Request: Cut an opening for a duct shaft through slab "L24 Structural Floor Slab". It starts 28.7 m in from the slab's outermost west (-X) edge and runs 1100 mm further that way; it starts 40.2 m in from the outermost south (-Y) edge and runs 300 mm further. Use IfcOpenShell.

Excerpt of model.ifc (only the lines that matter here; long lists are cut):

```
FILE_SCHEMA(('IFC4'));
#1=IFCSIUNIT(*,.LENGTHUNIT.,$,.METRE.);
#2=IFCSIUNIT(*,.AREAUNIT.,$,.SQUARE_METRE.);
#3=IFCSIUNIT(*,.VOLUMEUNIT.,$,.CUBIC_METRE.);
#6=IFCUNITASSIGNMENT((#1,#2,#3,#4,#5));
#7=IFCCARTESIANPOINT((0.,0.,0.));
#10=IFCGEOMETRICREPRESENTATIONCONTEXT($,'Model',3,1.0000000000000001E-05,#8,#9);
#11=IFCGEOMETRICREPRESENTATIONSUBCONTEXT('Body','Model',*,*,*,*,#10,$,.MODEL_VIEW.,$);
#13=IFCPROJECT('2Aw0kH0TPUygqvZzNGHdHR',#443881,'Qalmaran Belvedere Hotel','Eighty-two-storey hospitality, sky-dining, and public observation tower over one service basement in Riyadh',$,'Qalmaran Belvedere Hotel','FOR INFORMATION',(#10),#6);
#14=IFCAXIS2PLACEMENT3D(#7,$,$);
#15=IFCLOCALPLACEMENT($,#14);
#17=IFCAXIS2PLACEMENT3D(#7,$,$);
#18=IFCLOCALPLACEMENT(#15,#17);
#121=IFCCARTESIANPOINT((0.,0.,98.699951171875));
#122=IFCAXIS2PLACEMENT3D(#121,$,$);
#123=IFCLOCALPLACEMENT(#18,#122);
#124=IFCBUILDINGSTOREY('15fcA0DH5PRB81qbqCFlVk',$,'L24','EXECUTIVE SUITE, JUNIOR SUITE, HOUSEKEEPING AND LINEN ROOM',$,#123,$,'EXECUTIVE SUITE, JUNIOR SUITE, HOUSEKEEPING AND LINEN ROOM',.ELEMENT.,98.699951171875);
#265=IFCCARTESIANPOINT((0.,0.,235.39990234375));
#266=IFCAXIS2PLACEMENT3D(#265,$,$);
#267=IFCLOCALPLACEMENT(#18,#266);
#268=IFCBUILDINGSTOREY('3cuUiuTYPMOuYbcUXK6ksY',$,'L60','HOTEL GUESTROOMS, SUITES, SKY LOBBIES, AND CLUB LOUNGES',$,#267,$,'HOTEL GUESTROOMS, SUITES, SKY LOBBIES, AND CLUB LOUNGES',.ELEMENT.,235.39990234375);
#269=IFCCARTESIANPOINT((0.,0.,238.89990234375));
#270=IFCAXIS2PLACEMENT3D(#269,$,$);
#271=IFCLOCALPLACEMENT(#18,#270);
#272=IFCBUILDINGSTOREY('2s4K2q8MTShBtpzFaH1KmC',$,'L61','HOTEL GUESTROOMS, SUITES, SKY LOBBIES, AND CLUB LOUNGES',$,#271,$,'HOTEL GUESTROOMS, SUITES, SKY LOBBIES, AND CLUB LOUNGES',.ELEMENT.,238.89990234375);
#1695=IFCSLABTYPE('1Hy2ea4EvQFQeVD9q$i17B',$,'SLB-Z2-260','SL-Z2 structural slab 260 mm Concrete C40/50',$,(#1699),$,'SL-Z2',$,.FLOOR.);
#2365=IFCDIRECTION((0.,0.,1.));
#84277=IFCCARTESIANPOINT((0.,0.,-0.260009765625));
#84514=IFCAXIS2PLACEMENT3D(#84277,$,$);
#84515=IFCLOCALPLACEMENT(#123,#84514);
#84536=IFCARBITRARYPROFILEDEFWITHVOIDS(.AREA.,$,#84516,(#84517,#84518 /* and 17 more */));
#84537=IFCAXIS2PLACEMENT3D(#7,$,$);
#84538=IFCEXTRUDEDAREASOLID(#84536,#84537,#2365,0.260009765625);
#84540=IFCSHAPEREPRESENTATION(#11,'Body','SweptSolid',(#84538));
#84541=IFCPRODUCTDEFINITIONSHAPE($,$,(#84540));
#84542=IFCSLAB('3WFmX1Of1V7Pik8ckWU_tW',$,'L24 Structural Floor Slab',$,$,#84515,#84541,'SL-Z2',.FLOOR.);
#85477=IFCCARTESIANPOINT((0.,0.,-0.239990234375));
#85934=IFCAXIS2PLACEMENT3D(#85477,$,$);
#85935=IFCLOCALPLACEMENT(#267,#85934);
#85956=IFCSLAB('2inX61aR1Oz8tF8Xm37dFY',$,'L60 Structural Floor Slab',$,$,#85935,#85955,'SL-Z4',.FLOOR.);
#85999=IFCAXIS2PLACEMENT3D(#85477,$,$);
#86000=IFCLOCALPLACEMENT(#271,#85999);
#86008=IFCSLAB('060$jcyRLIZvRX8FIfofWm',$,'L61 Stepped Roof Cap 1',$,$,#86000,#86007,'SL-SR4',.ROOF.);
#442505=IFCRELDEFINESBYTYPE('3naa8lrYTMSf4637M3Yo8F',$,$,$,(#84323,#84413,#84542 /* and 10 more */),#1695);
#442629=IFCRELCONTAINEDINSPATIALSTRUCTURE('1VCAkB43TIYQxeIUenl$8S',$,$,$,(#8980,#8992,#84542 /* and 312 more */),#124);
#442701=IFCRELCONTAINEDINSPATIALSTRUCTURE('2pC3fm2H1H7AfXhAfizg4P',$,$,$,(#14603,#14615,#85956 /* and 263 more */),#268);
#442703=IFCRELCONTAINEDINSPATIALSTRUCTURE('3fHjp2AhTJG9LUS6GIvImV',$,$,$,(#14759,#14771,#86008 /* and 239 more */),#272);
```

```python
import numpy as np
import ifcopenshell
import ifcopenshell.api.feature
import ifcopenshell.api.geometry
import ifcopenshell.api.root
import ifcopenshell.geom
import ifcopenshell.util.placement
import ifcopenshell.util.representation
import ifcopenshell.util.shape
import ifcopenshell.util.unit

model = ifcopenshell.open("model.ifc")
unit_scale = ifcopenshell.util.unit.calculate_unit_scale(model)
settings = ifcopenshell.geom.settings()


def volume(element):
    """Net volume in cubic metres, openings subtracted."""
    shape = ifcopenshell.geom.create_shape(settings, element)
    return ifcopenshell.util.shape.get_volume(shape.geometry)


slab = model.by_id(84542)
before = volume(slab)

# Extent in the slab's own axes, in metres. The edges named are its -X and -Y sides.
slab_shape = ifcopenshell.geom.create_shape(settings, slab)
vertices = ifcopenshell.util.shape.get_vertices(slab_shape.geometry)
x_min, y_min, bottom = vertices.min(axis=0)
top = vertices[:, 2].max()

opening = ifcopenshell.api.root.create_entity(model, ifc_class="IfcOpeningElement", name="Duct shaft opening", predefined_type="OPENING")
context = ifcopenshell.util.representation.get_context(model, "Model", "Body", "MODEL_VIEW")
width, depth = 1.1, 0.3
outline = [(0.0, 0.0), (width, 0.0), (width, depth), (0.0, depth), (0.0, 0.0)]
# Overshoot both faces by 50 mm so the cut is clean.
shape = ifcopenshell.api.geometry.add_slab_representation(
    model, context=context, depth=top - bottom + 0.1, polyline=outline
)
ifcopenshell.api.geometry.assign_representation(model, product=opening, representation=shape)

matrix = ifcopenshell.util.placement.get_local_placement(slab.ObjectPlacement)
matrix[:, 3] = matrix @ np.append(np.array([x_min + 28.7, y_min + 40.2, bottom - 0.05]) / unit_scale, 1.0)
ifcopenshell.api.geometry.edit_object_placement(model, product=opening, matrix=matrix, is_si=False)
ifcopenshell.api.feature.add_feature(model, feature=opening, element=slab)

after = volume(slab)

print(f"slab volume {before:.3f} -> {after:.3f} m3")

model.write("model-out.ifc")
```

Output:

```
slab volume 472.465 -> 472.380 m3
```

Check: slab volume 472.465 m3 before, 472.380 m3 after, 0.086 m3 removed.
